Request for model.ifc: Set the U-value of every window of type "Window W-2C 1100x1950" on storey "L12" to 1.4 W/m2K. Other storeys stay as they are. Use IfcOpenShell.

First a look at what the model holds.

```python
import ifcopenshell
import ifcopenshell.util.element

model = ifcopenshell.open("model.ifc")
print(model.schema)
storey = next(s for s in model.by_type("IfcBuildingStorey") if s.Name == "L12")
windows = [e for e in ifcopenshell.util.element.get_decomposition(storey) if e.is_a("IfcWindow")]
seen = {}
for e in windows:
    element_type = ifcopenshell.util.element.get_type(e)
    key = (element_type.Name if element_type != e and element_type else None, ifcopenshell.util.element.get_pset(e, "Pset_WindowCommon", "ThermalTransmittance"))
    seen[key] = seen.get(key, 0) + 1
for (name, value), count in sorted(seen.items(), key=str):
    print(count, "x", name, "|", value)
```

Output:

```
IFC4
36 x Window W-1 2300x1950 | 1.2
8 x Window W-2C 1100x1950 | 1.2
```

```python
import ifcopenshell
import ifcopenshell.api.pset
import ifcopenshell.util.element

model = ifcopenshell.open("model.ifc")

storey = next(s for s in model.by_type("IfcBuildingStorey") if s.Name == "L12")
windows = [e for e in ifcopenshell.util.element.get_decomposition(storey) if e.is_a("IfcWindow")]

count = 0
for e in windows:
    element_type = ifcopenshell.util.element.get_type(e)
    if element_type in (None, e) or element_type.Name != "Window W-2C 1100x1950":
        continue
    found = ifcopenshell.util.element.get_pset(e, "Pset_WindowCommon", should_inherit=False)
    if found:
        pset = model.by_id(found["id"])
        if len(ifcopenshell.util.element.get_elements_by_pset(pset)) > 1:
            pset = ifcopenshell.api.pset.unshare_pset(model, products=[e], pset=pset)[0]
    else:
        pset = ifcopenshell.api.pset.add_pset(model, product=e, name="Pset_WindowCommon")
    ifcopenshell.api.pset.edit_pset(model, pset=pset, properties={"ThermalTransmittance": 1.4})
    count += 1

print(count, "windows updated")

model.write("model_edited.ifc")
```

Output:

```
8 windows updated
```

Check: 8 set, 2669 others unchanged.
